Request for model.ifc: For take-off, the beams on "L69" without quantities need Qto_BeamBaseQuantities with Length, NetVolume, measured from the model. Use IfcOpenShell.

First a look at what the model holds.

```python
import ifcopenshell
import ifcopenshell.util.element
import ifcopenshell.util.unit

model = ifcopenshell.open("model.ifc")
print(model.schema)
for unit_type in ("LENGTHUNIT", "AREAUNIT", "VOLUMEUNIT"):
    print(unit_type, ifcopenshell.util.unit.calculate_unit_scale(model, unit_type))
storey = next(s for s in model.by_type("IfcBuildingStorey") if s.Name == "L69")
beams = [e for e in ifcopenshell.util.element.get_decomposition(storey) if e.is_a("IfcBeam")]
for e in sorted(beams, key=lambda e: e.id()):
    print(e.id(), e.is_a(), e.Name, list(ifcopenshell.util.element.get_psets(e, qtos_only=True)), sep=" | ")
```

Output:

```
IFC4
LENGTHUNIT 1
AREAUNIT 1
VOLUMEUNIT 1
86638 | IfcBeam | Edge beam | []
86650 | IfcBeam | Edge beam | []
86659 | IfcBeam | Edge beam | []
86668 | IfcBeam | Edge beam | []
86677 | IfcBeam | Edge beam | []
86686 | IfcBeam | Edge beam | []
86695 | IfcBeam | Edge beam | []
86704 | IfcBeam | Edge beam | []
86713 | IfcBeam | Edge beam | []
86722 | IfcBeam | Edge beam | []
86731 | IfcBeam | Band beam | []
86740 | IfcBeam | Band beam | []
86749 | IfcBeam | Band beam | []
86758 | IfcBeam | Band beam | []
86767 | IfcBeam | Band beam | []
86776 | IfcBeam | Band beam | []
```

```python
import ifcopenshell
import ifcopenshell.api.pset
import ifcopenshell.geom
import ifcopenshell.util.element
import ifcopenshell.util.shape
import ifcopenshell.util.unit

model = ifcopenshell.open("model.ifc")
unit_scale = ifcopenshell.util.unit.calculate_unit_scale(model)
volume_scale = ifcopenshell.util.unit.calculate_unit_scale(model, "VOLUMEUNIT")
settings = ifcopenshell.geom.settings()

storey = next(s for s in model.by_type("IfcBuildingStorey") if s.Name == "L69")
beams = [e for e in ifcopenshell.util.element.get_decomposition(storey) if e.is_a("IfcBeam")]

for e in sorted(beams, key=lambda e: e.id()):
    if ifcopenshell.util.element.get_psets(e, qtos_only=True, should_inherit=False):
        continue
    # Geometry comes back in metres, in the element's own axes.
    shape = ifcopenshell.geom.create_shape(settings, e)
    values = {
        "Length": ifcopenshell.util.shape.get_max_xyz(shape.geometry) / unit_scale,
        "NetVolume": ifcopenshell.util.shape.get_volume(shape.geometry) / volume_scale,
    }
    qto = ifcopenshell.api.pset.add_qto(model, product=e, name="Qto_BeamBaseQuantities")
    ifcopenshell.api.pset.edit_qto(model, qto=qto, properties=values)
    print(e.id(), {k: round(v, 3) for k, v in values.items()})

model.write("model_edited.ifc")
```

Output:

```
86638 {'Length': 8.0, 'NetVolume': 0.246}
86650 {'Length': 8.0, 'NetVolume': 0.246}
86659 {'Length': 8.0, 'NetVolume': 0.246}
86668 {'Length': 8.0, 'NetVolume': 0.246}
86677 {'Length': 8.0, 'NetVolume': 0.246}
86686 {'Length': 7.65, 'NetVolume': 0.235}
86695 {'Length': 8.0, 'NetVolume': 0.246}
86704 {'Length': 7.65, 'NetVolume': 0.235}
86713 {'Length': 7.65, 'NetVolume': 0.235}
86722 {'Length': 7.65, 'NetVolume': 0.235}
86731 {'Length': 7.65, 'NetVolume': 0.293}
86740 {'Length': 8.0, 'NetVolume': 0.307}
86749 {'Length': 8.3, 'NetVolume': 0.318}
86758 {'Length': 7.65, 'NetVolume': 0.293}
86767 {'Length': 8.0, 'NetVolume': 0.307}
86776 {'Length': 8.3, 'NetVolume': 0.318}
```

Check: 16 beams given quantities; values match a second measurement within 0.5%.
